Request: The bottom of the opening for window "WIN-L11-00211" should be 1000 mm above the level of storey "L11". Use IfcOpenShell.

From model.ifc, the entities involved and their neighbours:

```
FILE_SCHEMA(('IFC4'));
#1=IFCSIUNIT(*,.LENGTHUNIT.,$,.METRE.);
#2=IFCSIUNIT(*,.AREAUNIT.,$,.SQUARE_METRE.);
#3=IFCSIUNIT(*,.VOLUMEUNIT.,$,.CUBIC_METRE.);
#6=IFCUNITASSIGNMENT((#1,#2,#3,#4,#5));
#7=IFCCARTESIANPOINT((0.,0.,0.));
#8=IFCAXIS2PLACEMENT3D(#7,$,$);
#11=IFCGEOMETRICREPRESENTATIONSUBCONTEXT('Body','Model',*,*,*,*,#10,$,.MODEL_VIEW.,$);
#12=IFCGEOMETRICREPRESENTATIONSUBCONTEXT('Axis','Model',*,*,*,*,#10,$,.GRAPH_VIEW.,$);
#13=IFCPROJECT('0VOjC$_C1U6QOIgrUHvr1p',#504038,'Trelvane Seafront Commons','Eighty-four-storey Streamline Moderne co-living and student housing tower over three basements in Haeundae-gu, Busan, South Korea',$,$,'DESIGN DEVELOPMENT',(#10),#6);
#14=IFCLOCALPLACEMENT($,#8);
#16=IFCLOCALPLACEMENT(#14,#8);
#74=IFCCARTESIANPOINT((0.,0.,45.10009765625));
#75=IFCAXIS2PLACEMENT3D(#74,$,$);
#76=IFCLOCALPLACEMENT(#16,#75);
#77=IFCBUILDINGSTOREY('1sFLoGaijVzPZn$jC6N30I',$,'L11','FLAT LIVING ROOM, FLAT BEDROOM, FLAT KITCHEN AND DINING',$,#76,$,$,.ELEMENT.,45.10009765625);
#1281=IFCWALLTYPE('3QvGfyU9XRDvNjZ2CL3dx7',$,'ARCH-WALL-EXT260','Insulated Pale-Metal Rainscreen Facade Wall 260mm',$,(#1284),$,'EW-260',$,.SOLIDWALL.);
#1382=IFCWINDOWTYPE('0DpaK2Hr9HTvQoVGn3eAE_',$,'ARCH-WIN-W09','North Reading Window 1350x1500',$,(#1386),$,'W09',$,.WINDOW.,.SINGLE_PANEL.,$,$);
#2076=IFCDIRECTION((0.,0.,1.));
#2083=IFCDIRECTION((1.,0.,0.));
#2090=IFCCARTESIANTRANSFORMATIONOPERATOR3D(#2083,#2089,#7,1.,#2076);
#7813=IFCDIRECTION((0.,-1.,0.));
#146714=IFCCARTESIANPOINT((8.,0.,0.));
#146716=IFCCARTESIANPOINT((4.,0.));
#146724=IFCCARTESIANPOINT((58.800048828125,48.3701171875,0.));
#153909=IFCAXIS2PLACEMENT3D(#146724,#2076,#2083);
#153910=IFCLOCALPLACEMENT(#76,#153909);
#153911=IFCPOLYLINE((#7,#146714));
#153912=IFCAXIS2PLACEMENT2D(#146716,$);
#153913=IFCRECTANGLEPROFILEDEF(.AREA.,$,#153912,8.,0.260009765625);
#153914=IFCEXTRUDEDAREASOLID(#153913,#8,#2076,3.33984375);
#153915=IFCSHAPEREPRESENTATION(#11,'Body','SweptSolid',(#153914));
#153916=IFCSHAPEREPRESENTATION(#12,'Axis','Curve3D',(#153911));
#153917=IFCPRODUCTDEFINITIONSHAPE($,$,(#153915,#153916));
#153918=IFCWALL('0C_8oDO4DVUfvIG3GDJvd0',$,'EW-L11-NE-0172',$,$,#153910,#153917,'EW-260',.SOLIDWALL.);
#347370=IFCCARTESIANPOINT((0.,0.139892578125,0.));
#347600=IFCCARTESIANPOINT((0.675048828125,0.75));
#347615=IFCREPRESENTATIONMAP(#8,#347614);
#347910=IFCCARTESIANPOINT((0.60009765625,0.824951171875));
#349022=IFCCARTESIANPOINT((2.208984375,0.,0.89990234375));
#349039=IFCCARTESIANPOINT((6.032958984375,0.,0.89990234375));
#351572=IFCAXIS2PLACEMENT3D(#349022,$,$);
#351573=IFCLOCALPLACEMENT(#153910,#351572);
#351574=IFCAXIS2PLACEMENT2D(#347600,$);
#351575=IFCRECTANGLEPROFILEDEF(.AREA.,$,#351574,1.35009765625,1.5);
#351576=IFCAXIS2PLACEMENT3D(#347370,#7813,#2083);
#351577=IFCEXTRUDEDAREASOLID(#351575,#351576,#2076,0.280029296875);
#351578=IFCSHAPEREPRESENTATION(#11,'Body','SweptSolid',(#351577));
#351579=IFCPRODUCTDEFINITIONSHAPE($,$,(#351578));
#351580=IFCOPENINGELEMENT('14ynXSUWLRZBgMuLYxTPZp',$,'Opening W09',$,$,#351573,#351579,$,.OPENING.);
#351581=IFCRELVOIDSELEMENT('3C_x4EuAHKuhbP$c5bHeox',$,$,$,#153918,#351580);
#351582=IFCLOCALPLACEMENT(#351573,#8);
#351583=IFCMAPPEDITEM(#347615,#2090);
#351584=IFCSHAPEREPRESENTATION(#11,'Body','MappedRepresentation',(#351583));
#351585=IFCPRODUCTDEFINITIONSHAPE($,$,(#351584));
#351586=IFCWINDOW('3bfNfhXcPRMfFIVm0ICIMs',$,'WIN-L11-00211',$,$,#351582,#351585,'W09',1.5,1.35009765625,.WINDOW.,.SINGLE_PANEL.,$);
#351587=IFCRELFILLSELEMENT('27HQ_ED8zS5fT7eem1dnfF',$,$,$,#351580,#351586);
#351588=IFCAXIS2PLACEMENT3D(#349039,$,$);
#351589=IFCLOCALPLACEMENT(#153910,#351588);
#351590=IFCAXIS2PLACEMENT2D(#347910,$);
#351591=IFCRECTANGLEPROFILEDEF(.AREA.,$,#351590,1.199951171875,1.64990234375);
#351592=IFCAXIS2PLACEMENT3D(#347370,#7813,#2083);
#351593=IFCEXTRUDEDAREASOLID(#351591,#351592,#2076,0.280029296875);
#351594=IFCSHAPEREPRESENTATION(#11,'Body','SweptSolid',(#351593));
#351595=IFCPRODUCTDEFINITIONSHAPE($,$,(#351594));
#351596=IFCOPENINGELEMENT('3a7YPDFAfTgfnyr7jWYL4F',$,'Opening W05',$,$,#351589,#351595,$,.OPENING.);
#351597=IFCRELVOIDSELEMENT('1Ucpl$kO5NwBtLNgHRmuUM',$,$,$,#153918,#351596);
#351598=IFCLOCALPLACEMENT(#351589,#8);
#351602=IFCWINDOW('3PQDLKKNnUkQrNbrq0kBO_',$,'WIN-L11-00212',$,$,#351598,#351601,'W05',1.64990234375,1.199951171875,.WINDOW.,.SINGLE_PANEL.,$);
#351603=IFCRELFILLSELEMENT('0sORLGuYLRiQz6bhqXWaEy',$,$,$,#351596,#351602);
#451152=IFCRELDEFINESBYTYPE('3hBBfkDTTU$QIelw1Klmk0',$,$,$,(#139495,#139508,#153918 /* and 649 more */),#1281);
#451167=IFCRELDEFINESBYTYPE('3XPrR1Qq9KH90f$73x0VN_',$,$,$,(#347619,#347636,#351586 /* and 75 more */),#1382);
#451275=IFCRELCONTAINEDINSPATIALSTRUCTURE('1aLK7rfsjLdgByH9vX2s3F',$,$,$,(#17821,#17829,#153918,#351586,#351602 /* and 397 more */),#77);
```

```python
import numpy as np
import ifcopenshell
import ifcopenshell.api.geometry
import ifcopenshell.geom
import ifcopenshell.util.element
import ifcopenshell.util.placement
import ifcopenshell.util.shape
import ifcopenshell.util.unit

model = ifcopenshell.open("model.ifc")
unit_scale = ifcopenshell.util.unit.calculate_unit_scale(model)

window = model.by_guid("3bfNfhXcPRMfFIVm0ICIMs")
opening = window.FillsVoids[0].RelatingOpeningElement
storey = ifcopenshell.util.element.get_container(window, ifc_class="IfcBuildingStorey")
level = ifcopenshell.util.placement.get_local_placement(storey.ObjectPlacement)[2, 3]

# The opening's origin need not be at the sill, so measure its lowest point.
shape = ifcopenshell.geom.create_shape(ifcopenshell.geom.settings(), opening)
bottom = ifcopenshell.util.shape.get_shape_bottom_elevation(shape, shape.geometry) / unit_scale
dz = level + 1.0 - bottom

shift = np.array([0.0, 0.0, dz])
# The window is placed relative to its opening, so it follows when the opening moves.
matrix = ifcopenshell.util.placement.get_local_placement(opening.ObjectPlacement)
matrix[:3, 3] += shift
ifcopenshell.api.geometry.edit_object_placement(
    model, product=opening, matrix=matrix, is_si=False, should_transform_children=True
)

print(f"moved by {dz * unit_scale:+.3f} m")

model.write("model_updated.ifc")
```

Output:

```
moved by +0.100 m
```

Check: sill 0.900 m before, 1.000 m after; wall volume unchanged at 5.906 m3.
